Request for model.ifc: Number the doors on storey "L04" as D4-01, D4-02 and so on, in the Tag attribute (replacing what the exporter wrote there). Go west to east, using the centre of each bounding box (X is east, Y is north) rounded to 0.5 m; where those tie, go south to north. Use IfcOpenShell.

First a look at what the model holds.

```python
import ifcopenshell
import ifcopenshell.util.element
import ifcopenshell.util.placement

model = ifcopenshell.open("model.ifc")
print(model.schema)
storey = next(s for s in model.by_type("IfcBuildingStorey") if s.Name == "L04")
doors = [e for e in ifcopenshell.util.element.get_decomposition(storey) if e.is_a("IfcDoor")]
for e in sorted(doors, key=lambda e: e.id()):
    origin = ifcopenshell.util.placement.get_local_placement(e.ObjectPlacement)[:3, 3]
    print(e.id(), e.Tag, e.Name, origin.round(2) + 0.0, sep=" | ")
```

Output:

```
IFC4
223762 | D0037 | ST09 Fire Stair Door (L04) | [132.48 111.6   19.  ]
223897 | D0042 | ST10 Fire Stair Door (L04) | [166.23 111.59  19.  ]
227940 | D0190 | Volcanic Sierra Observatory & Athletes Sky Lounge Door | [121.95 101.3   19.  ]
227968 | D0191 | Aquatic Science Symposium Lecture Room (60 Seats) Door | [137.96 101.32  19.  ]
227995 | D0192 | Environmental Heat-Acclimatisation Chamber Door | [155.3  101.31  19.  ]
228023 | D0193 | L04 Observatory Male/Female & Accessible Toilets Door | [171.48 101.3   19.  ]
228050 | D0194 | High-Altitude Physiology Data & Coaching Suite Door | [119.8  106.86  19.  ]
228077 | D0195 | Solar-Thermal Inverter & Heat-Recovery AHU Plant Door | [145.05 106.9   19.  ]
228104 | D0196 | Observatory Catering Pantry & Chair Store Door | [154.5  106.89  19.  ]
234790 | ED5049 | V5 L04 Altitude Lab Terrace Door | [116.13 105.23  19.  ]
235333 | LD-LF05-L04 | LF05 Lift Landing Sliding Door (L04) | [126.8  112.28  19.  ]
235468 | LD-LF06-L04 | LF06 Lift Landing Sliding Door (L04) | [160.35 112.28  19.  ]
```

```python
import ifcopenshell
import ifcopenshell.geom
import ifcopenshell.util.element
import ifcopenshell.util.shape

model = ifcopenshell.open("model.ifc")
settings = ifcopenshell.geom.settings()
settings.set("use-world-coords", True)


def centre(element):
    shape = ifcopenshell.geom.create_shape(settings, element)
    return ifcopenshell.util.shape.get_bbox_centroid(shape.geometry)


storey = next(s for s in model.by_type("IfcBuildingStorey") if s.Name == "L04")
doors = [e for e in ifcopenshell.util.element.get_decomposition(storey) if e.is_a("IfcDoor")]

# Insertion points can sit at a corner or the storey origin, so sort by the geometry (in metres).
centres = {e: centre(e) for e in doors}
doors.sort(key=lambda e: (round(centres[e][0] / 0.5), centres[e][1]))

for i, e in enumerate(doors, start=1):
    number = f"D4-{i:02d}"
    e.Tag = number
    print(e.id(), number)

model.write("model_v2.ifc")
```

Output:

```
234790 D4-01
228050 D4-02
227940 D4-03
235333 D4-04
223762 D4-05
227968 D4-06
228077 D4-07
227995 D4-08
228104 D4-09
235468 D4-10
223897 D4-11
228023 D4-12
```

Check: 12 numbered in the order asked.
